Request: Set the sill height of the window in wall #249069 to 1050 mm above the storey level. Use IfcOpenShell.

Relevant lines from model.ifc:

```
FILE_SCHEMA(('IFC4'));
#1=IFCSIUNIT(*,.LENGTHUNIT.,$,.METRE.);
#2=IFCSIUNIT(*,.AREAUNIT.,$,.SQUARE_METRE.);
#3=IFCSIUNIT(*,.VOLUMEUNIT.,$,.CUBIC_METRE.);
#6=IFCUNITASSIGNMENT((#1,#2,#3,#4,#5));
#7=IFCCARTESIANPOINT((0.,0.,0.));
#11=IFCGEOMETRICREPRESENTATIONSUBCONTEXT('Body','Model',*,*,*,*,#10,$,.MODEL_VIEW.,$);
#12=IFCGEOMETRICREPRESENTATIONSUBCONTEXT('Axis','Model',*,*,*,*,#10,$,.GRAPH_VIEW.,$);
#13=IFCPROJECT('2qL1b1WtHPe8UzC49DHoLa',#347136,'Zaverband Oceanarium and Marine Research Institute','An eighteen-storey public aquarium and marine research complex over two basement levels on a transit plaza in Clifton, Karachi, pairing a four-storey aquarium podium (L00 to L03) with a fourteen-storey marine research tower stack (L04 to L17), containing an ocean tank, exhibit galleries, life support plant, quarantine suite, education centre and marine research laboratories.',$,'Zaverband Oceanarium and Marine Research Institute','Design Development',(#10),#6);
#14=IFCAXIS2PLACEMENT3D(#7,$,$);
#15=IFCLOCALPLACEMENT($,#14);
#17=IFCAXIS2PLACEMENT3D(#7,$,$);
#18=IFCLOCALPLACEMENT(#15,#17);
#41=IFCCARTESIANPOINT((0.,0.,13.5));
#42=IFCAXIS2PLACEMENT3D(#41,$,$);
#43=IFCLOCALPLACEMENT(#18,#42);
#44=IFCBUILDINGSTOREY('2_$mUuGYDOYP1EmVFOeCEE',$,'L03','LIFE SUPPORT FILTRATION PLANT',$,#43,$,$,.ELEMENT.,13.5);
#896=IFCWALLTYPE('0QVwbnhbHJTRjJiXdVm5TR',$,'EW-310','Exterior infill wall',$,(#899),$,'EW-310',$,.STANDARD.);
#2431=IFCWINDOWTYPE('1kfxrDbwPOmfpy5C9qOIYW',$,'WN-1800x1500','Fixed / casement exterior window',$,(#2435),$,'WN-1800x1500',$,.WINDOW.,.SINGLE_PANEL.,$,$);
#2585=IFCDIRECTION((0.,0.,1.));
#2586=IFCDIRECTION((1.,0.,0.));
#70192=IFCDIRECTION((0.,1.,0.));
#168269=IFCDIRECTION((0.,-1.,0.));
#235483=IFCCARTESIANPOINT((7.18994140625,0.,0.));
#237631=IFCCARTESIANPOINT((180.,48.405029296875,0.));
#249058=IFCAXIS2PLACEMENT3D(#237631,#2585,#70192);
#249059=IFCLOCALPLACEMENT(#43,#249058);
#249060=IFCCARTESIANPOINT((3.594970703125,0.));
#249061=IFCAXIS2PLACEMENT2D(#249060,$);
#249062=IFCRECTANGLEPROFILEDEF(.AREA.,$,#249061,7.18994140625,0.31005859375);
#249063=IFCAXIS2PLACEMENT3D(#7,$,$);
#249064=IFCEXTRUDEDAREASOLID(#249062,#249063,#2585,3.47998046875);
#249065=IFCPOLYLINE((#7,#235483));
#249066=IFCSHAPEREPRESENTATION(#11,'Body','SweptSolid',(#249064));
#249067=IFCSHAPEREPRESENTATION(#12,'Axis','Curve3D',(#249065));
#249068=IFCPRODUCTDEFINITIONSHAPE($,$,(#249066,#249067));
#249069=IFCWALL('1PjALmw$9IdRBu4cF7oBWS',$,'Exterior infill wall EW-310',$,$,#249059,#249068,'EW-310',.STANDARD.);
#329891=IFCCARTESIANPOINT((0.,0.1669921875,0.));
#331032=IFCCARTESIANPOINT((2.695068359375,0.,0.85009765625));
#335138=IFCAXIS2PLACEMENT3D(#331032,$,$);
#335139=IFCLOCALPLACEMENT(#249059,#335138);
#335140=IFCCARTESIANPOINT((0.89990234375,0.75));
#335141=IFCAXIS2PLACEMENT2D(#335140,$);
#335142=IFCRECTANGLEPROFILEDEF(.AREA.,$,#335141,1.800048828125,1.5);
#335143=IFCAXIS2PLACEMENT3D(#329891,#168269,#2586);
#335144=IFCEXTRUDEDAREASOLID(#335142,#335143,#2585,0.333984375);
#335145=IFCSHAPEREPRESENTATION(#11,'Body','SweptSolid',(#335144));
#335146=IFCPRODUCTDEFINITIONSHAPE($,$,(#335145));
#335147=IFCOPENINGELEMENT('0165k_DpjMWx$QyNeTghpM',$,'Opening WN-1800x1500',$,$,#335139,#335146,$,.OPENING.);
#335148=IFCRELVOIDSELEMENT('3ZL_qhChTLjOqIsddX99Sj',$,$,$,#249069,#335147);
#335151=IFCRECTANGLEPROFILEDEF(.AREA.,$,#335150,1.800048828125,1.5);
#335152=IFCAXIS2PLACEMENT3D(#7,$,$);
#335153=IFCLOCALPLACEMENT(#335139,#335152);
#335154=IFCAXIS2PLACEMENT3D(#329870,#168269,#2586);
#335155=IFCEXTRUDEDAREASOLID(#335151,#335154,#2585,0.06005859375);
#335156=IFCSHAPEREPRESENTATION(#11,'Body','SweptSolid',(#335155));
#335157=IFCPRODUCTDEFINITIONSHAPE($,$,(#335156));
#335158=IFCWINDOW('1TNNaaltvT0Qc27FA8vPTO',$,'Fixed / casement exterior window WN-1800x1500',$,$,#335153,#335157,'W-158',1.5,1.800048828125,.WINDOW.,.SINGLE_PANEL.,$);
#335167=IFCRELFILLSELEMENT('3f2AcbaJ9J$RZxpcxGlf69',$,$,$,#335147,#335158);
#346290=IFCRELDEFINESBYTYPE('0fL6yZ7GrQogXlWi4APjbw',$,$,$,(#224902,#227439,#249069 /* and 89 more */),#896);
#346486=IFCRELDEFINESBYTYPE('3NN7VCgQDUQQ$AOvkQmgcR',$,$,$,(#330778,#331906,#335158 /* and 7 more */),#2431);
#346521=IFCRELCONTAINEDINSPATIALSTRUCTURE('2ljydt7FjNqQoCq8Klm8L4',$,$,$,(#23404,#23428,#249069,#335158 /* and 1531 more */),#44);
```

```python
import numpy as np
import ifcopenshell
import ifcopenshell.api.geometry
import ifcopenshell.geom
import ifcopenshell.util.element
import ifcopenshell.util.placement
import ifcopenshell.util.shape
import ifcopenshell.util.unit

model = ifcopenshell.open("model.ifc")
unit_scale = ifcopenshell.util.unit.calculate_unit_scale(model)

window = model.by_guid("1TNNaaltvT0Qc27FA8vPTO")
opening = window.FillsVoids[0].RelatingOpeningElement
storey = ifcopenshell.util.element.get_container(window, ifc_class="IfcBuildingStorey")
level = ifcopenshell.util.placement.get_local_placement(storey.ObjectPlacement)[2, 3]

# The opening's origin need not be at the sill, so measure its lowest point.
shape = ifcopenshell.geom.create_shape(ifcopenshell.geom.settings(), opening)
bottom = ifcopenshell.util.shape.get_shape_bottom_elevation(shape, shape.geometry) / unit_scale
dz = level + 1.05 - bottom

shift = np.array([0.0, 0.0, dz])
# The window is placed relative to its opening, so it follows when the opening moves.
matrix = ifcopenshell.util.placement.get_local_placement(opening.ObjectPlacement)
matrix[:3, 3] += shift
ifcopenshell.api.geometry.edit_object_placement(
    model, product=opening, matrix=matrix, is_si=False, should_transform_children=True
)

print(f"moved by {dz * unit_scale:+.3f} m")

model.write("model_v2.ifc")
```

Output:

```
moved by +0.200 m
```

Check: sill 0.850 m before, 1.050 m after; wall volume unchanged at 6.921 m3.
